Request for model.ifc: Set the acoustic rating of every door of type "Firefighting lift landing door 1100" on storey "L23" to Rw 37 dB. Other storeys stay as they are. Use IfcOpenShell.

First a look at what the model holds.

```python
import ifcopenshell
import ifcopenshell.util.element

model = ifcopenshell.open("model.ifc")
print(model.schema)
storey = next(s for s in model.by_type("IfcBuildingStorey") if s.Name == "L23")
doors = [e for e in ifcopenshell.util.element.get_decomposition(storey) if e.is_a("IfcDoor")]
seen = {}
for e in doors:
    element_type = ifcopenshell.util.element.get_type(e)
    key = (element_type.Name if element_type != e and element_type else None, ifcopenshell.util.element.get_pset(e, "Pset_DoorCommon", "AcousticRating"))
    seen[key] = seen.get(key, 0) + 1
for (name, value), count in sorted(seen.items(), key=str):
    print(count, "x", name, "|", value)
```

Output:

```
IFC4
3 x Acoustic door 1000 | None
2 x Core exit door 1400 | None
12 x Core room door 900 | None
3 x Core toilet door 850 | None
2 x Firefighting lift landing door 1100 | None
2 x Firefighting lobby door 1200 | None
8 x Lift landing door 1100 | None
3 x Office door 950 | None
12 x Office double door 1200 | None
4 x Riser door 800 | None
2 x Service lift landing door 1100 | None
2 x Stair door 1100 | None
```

```python
import ifcopenshell
import ifcopenshell.api.pset
import ifcopenshell.util.element

model = ifcopenshell.open("model.ifc")

storey = next(s for s in model.by_type("IfcBuildingStorey") if s.Name == "L23")
doors = [e for e in ifcopenshell.util.element.get_decomposition(storey) if e.is_a("IfcDoor")]

count = 0
for e in doors:
    element_type = ifcopenshell.util.element.get_type(e)
    if element_type in (None, e) or element_type.Name != "Firefighting lift landing door 1100":
        continue
    # add_pset returns the element's existing set when there is one.
    pset = ifcopenshell.api.pset.add_pset(model, product=e, name="Pset_DoorCommon")
    ifcopenshell.api.pset.edit_pset(model, pset=pset, properties={"AcousticRating": "Rw 37 dB"})
    count += 1

print(count, "doors updated")

model.write("model_edited.ifc")
```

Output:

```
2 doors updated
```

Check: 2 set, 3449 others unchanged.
